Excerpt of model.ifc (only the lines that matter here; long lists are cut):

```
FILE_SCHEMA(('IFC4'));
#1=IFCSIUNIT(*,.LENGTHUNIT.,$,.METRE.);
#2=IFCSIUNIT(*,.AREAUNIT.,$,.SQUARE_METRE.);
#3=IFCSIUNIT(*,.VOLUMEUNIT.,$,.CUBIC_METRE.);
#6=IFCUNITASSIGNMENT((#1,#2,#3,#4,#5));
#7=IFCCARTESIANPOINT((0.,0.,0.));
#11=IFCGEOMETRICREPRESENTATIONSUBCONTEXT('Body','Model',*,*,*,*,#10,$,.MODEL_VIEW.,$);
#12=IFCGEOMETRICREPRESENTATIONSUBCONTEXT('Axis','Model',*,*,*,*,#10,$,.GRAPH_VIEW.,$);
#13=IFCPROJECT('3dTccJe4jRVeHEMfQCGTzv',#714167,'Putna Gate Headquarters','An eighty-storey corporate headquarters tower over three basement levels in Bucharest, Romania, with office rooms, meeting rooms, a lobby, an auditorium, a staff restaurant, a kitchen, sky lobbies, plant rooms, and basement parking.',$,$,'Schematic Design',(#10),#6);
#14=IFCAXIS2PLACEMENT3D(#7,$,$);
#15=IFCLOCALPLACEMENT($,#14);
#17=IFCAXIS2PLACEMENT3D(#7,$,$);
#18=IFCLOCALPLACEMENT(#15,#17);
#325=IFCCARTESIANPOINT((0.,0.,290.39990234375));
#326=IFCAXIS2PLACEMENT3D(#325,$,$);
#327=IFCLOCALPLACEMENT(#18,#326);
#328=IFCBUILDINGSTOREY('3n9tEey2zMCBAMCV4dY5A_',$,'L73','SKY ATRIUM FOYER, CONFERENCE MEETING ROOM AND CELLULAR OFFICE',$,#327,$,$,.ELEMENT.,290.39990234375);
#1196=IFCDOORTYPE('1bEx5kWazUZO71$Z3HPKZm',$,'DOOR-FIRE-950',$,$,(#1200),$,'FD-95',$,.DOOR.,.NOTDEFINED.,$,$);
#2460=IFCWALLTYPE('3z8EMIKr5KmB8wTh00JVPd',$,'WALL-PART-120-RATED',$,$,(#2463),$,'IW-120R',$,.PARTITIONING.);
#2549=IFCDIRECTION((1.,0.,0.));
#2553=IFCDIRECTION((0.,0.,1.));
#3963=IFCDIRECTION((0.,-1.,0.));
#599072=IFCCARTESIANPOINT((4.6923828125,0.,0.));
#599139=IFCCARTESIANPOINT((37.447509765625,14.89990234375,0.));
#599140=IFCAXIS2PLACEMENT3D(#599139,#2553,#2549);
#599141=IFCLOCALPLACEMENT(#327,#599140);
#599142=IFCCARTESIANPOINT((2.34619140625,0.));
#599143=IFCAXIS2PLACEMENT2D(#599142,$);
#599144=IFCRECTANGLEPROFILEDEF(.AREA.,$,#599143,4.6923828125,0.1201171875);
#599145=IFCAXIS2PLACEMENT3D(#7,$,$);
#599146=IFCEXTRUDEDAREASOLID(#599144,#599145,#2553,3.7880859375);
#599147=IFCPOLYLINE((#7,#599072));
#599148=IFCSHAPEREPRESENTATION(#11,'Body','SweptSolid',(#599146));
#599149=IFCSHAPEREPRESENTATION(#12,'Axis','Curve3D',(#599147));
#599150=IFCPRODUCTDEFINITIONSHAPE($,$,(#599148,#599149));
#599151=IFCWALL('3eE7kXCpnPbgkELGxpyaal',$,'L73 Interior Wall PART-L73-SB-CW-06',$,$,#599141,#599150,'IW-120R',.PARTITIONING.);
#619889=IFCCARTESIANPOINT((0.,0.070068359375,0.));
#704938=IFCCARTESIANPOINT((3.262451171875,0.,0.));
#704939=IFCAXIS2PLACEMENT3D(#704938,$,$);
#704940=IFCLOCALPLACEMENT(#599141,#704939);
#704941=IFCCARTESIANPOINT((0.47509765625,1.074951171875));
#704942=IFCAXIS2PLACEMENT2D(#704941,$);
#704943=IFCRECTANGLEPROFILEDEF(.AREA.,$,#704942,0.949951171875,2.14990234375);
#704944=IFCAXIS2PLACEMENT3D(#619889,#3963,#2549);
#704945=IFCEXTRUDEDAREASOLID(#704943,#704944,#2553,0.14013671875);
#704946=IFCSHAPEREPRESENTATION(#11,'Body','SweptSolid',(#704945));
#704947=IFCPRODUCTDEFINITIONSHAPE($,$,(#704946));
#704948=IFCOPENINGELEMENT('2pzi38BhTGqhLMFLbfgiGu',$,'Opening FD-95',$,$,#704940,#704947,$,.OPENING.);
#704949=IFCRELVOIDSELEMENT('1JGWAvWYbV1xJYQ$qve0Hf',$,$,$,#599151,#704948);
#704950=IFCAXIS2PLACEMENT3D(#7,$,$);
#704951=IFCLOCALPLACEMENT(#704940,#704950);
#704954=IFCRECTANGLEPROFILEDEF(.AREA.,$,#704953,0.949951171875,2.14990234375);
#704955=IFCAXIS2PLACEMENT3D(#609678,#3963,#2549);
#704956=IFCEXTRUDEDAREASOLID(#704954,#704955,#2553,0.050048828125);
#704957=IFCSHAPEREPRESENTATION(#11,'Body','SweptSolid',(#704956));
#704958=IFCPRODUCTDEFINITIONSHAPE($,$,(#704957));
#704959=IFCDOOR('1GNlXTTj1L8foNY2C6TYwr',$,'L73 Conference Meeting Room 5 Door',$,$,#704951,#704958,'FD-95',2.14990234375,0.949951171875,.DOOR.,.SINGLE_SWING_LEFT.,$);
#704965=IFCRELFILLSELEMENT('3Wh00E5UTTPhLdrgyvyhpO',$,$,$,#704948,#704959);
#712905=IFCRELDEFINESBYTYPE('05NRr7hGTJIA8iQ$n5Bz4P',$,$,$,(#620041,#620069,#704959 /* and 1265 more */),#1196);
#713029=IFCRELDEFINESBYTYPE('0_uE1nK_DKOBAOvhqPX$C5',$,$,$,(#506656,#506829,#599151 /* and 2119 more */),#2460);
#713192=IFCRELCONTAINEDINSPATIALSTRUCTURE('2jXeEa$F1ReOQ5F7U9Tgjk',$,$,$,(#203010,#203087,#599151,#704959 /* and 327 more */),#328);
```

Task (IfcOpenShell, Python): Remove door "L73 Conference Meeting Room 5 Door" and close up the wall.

```python
import ifcopenshell
import ifcopenshell.api.feature
import ifcopenshell.api.root
import ifcopenshell.geom
import ifcopenshell.util.shape

model = ifcopenshell.open("model.ifc")
settings = ifcopenshell.geom.settings()


def volume(element):
    """Net volume in cubic metres, openings subtracted."""
    shape = ifcopenshell.geom.create_shape(settings, element)
    return ifcopenshell.util.shape.get_volume(shape.geometry)


door = model.by_id(704959)
opening = door.FillsVoids[0].RelatingOpeningElement
wall = opening.VoidsElements[0].RelatingBuildingElement
before = volume(wall)

ifcopenshell.api.root.remove_product(model, product=door)
ifcopenshell.api.feature.remove_feature(model, feature=opening)

after = volume(wall)

print(f"wall volume {before:.3f} -> {after:.3f} m3")

model.write("model_rev.ifc")
```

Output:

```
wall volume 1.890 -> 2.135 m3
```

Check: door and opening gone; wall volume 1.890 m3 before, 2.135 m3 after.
